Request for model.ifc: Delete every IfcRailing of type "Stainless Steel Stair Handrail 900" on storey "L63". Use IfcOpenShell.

First a look at what the model holds.

```python
import ifcopenshell
import ifcopenshell.util.element

model = ifcopenshell.open("model.ifc")
print(model.schema)
storey = next(s for s in model.by_type("IfcBuildingStorey") if s.Name == "L63")
railings = [e for e in ifcopenshell.util.element.get_decomposition(storey) if e.is_a("IfcRailing")]
seen = {}
for e in railings:
    element_type = ifcopenshell.util.element.get_type(e)
    name = element_type.Name if element_type not in (None, e) else None
    seen[name] = seen.get(name, 0) + 1
for name, count in sorted(seen.items(), key=str):
    print(count, "x", name)
```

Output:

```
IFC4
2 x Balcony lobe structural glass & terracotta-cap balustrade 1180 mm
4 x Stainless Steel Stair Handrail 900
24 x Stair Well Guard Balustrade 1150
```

```python
import ifcopenshell
import ifcopenshell.api.root
import ifcopenshell.util.element

model = ifcopenshell.open("model.ifc")

storey = next(s for s in model.by_type("IfcBuildingStorey") if s.Name == "L63")
railings = [e for e in ifcopenshell.util.element.get_decomposition(storey) if e.is_a("IfcRailing")]
targets = [e for e in railings if (t := ifcopenshell.util.element.get_type(e)) not in (None, e) and t.Name == "Stainless Steel Stair Handrail 900"]

for e in targets:
    ifcopenshell.api.root.remove_product(model, product=e)
print(len(targets), "removed")

model.write("model_updated.ifc")
```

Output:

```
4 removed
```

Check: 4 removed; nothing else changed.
